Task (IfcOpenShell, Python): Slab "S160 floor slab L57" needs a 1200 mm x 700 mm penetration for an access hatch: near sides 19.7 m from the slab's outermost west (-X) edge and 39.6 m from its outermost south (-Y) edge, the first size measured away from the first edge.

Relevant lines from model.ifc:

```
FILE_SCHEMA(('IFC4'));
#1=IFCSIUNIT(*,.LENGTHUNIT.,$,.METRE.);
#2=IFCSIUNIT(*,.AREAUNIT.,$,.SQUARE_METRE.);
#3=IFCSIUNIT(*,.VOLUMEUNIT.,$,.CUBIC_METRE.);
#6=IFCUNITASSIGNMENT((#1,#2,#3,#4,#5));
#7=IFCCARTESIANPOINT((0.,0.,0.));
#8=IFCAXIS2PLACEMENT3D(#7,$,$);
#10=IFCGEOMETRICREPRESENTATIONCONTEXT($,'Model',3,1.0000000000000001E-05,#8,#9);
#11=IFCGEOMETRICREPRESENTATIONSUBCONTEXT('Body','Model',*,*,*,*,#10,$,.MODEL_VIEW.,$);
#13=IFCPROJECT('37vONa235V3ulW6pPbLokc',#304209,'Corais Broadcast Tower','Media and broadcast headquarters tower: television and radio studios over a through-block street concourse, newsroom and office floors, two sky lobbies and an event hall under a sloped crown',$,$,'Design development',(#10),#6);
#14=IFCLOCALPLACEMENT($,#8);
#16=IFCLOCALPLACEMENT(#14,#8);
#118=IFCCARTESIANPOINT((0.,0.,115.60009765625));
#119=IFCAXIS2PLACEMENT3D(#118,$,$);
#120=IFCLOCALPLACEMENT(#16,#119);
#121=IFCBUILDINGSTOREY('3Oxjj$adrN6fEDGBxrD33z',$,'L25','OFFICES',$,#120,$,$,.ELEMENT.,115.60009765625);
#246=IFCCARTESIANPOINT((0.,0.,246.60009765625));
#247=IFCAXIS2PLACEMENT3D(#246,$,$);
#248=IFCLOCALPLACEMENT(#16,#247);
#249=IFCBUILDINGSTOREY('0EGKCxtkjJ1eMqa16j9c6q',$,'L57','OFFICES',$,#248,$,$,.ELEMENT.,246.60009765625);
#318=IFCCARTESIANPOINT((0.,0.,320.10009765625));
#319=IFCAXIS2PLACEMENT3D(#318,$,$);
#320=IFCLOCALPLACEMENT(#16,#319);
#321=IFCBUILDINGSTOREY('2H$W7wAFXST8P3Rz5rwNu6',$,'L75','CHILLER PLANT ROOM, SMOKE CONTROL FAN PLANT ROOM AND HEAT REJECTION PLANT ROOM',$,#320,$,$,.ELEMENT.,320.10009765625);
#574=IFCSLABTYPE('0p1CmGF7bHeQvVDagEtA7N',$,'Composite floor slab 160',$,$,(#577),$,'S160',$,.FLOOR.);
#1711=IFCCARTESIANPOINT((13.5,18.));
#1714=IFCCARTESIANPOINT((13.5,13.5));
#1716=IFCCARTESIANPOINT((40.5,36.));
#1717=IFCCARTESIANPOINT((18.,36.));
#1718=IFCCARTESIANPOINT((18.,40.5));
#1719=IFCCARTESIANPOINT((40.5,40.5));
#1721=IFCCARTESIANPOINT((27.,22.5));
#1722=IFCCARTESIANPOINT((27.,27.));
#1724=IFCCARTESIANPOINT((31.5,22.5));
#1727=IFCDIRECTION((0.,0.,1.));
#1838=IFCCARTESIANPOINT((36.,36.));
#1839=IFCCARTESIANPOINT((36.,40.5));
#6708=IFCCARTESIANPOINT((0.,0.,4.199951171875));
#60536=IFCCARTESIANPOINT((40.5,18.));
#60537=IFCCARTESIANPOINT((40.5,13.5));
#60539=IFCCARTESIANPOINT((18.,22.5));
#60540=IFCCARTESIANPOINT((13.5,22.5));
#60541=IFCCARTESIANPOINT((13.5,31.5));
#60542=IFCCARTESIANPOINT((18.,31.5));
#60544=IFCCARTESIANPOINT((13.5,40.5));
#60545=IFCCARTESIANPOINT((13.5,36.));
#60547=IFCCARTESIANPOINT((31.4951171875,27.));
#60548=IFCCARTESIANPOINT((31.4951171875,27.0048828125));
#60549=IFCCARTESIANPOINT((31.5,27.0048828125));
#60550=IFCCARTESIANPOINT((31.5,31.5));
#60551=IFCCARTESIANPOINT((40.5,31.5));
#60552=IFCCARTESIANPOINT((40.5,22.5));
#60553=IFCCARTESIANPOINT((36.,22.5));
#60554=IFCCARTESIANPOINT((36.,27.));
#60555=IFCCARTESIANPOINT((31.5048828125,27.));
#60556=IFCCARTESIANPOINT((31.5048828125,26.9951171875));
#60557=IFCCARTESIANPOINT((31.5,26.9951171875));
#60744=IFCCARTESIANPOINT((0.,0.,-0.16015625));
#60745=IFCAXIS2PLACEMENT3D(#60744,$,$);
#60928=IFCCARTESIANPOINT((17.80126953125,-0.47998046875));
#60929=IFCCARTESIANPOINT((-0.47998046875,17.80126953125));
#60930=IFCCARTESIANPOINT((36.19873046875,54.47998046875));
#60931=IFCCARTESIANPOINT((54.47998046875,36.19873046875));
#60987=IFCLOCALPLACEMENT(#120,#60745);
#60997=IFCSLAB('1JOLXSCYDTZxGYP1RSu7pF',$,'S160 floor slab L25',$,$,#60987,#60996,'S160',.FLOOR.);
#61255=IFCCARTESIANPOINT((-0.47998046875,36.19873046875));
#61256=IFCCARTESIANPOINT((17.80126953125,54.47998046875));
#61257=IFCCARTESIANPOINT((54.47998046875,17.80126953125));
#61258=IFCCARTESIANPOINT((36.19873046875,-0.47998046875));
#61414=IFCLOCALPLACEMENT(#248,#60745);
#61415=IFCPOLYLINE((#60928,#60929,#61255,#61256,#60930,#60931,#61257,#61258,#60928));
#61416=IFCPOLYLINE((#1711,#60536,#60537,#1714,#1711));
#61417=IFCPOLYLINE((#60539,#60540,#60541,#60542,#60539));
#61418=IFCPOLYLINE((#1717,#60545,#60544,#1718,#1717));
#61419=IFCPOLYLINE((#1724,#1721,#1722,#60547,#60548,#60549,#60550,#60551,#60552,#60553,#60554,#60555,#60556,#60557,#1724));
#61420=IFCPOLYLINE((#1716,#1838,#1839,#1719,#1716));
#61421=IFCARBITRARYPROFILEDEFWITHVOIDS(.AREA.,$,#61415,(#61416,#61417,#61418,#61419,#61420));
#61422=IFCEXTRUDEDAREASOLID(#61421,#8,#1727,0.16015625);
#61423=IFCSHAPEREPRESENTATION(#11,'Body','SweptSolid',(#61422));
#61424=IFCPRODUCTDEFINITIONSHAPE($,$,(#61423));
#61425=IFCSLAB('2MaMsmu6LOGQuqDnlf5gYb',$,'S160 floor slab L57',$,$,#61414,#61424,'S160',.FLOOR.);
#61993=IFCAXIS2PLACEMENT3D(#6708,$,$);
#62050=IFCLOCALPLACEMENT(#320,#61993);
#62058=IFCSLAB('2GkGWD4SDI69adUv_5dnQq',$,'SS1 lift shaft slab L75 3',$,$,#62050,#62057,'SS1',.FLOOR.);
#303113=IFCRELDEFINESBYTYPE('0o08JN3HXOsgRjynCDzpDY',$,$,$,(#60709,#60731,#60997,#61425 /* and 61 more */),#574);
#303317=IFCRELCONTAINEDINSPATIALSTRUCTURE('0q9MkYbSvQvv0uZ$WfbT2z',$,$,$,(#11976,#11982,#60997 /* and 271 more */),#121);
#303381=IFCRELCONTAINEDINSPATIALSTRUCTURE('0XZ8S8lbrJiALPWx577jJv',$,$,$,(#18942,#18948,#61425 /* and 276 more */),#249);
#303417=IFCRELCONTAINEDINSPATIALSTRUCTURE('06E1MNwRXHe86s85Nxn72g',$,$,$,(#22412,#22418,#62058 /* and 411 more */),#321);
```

```python
import numpy as np
import ifcopenshell
import ifcopenshell.api.feature
import ifcopenshell.api.geometry
import ifcopenshell.api.root
import ifcopenshell.geom
import ifcopenshell.util.placement
import ifcopenshell.util.representation
import ifcopenshell.util.shape
import ifcopenshell.util.unit

model = ifcopenshell.open("model.ifc")
unit_scale = ifcopenshell.util.unit.calculate_unit_scale(model)
settings = ifcopenshell.geom.settings()


def volume(element):
    """Net volume in cubic metres, openings subtracted."""
    shape = ifcopenshell.geom.create_shape(settings, element)
    return ifcopenshell.util.shape.get_volume(shape.geometry)


slab = model.by_guid("2MaMsmu6LOGQuqDnlf5gYb")
before = volume(slab)

# Extent in the slab's own axes, in metres. The edges named are its -X and -Y sides.
slab_shape = ifcopenshell.geom.create_shape(settings, slab)
vertices = ifcopenshell.util.shape.get_vertices(slab_shape.geometry)
x_min, y_min, bottom = vertices.min(axis=0)
top = vertices[:, 2].max()

opening = ifcopenshell.api.root.create_entity(model, ifc_class="IfcOpeningElement", name="Access hatch opening", predefined_type="OPENING")
context = ifcopenshell.util.representation.get_context(model, "Model", "Body", "MODEL_VIEW")
width, depth = 1.2, 0.7
outline = [(0.0, 0.0), (width, 0.0), (width, depth), (0.0, depth), (0.0, 0.0)]
# Overshoot both faces by 50 mm so the cut is clean.
shape = ifcopenshell.api.geometry.add_slab_representation(
    model, context=context, depth=top - bottom + 0.1, polyline=outline
)
ifcopenshell.api.geometry.assign_representation(model, product=opening, representation=shape)

matrix = ifcopenshell.util.placement.get_local_placement(slab.ObjectPlacement)
matrix[:, 3] = matrix @ np.append(np.array([x_min + 19.7, y_min + 39.6, bottom - 0.05]) / unit_scale, 1.0)
ifcopenshell.api.geometry.edit_object_placement(model, product=opening, matrix=matrix, is_si=False)
ifcopenshell.api.feature.add_feature(model, feature=opening, element=slab)

after = volume(slab)

print(f"slab volume {before:.3f} -> {after:.3f} m3")

model.write("model_edited.ifc")
```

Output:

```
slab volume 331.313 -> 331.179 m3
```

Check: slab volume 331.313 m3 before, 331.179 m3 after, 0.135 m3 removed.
